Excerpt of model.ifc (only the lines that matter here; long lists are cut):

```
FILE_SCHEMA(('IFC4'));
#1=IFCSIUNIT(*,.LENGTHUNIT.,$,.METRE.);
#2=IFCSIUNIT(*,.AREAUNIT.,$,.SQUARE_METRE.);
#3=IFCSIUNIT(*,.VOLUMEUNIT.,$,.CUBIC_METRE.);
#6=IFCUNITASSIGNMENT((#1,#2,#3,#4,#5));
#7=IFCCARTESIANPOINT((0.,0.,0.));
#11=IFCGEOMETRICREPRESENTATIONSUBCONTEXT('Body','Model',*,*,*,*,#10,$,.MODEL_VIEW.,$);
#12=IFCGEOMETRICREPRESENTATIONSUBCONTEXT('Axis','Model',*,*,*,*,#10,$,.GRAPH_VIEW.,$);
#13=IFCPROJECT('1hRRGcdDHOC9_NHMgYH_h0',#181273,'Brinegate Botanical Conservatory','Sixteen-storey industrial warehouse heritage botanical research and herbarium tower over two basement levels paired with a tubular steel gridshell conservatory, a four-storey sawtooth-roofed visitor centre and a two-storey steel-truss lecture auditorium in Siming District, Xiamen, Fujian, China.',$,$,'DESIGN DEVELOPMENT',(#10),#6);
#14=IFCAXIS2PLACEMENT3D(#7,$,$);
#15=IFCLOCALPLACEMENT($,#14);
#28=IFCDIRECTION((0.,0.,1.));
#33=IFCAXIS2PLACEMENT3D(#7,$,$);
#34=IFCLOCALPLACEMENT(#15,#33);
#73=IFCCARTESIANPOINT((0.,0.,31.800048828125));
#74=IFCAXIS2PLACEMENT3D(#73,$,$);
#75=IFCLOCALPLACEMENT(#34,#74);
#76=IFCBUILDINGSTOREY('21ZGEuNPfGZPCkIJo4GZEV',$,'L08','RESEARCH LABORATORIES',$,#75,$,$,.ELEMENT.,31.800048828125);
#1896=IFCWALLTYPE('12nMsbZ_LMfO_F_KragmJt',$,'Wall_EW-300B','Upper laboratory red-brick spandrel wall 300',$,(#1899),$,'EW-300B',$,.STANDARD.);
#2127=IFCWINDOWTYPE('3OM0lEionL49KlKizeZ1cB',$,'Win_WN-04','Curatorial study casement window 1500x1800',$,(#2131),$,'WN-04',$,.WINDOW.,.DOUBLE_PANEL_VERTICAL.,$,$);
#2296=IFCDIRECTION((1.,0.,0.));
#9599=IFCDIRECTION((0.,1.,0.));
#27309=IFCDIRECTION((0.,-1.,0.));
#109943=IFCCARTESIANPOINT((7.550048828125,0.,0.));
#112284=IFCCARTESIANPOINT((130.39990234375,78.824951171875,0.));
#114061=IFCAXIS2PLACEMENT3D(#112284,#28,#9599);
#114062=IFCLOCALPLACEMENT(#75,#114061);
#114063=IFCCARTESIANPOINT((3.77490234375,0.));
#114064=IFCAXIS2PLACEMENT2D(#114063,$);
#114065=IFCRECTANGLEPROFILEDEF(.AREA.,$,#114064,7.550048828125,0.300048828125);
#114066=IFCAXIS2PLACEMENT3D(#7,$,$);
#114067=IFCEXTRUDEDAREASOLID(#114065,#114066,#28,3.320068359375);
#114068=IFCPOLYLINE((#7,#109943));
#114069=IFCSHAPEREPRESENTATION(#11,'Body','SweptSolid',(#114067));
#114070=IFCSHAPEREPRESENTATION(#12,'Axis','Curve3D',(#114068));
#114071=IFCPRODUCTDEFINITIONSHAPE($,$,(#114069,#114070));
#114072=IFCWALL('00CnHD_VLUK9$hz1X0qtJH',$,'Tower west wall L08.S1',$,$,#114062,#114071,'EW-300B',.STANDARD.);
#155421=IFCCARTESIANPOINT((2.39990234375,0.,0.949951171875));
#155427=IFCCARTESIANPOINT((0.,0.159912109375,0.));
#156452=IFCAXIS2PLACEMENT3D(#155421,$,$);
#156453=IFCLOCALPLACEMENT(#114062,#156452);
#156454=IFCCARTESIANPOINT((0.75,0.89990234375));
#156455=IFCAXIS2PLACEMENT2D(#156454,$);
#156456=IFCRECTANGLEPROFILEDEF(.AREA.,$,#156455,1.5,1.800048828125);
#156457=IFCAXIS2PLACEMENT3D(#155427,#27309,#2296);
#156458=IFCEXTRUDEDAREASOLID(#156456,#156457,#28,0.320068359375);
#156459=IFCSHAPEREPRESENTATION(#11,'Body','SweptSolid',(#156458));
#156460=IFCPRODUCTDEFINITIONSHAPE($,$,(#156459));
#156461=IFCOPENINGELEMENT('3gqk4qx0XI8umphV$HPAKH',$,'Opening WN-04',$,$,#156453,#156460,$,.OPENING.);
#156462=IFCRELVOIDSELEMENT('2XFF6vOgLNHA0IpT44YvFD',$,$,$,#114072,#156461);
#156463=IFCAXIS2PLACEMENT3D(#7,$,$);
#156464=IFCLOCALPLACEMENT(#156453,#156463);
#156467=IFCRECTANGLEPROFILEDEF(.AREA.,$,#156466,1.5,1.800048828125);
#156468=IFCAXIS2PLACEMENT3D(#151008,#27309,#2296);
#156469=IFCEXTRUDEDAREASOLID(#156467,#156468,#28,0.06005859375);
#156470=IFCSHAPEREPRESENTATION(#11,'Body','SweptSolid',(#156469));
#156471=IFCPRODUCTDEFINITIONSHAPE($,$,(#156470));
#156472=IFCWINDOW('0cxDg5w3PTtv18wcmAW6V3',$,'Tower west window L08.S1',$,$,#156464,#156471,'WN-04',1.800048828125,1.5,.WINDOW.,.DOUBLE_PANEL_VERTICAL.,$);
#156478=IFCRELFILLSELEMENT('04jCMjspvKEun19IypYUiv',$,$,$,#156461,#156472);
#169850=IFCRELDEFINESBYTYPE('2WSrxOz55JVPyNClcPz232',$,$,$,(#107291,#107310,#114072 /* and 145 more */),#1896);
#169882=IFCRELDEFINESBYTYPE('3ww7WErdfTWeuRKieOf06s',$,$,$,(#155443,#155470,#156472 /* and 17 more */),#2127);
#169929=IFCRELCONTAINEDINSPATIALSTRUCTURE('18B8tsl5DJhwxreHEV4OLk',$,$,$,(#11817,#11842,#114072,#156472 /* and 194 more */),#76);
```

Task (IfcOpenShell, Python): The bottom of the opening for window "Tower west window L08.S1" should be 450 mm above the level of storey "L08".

```python
import numpy as np
import ifcopenshell
import ifcopenshell.api.geometry
import ifcopenshell.geom
import ifcopenshell.util.element
import ifcopenshell.util.placement
import ifcopenshell.util.shape
import ifcopenshell.util.unit

model = ifcopenshell.open("model.ifc")
unit_scale = ifcopenshell.util.unit.calculate_unit_scale(model)

window = model.by_guid("0cxDg5w3PTtv18wcmAW6V3")
opening = window.FillsVoids[0].RelatingOpeningElement
storey = ifcopenshell.util.element.get_container(window, ifc_class="IfcBuildingStorey")
level = ifcopenshell.util.placement.get_local_placement(storey.ObjectPlacement)[2, 3]

# The opening's origin need not be at the sill, so measure its lowest point.
shape = ifcopenshell.geom.create_shape(ifcopenshell.geom.settings(), opening)
bottom = ifcopenshell.util.shape.get_shape_bottom_elevation(shape, shape.geometry) / unit_scale
dz = level + 0.45 - bottom

shift = np.array([0.0, 0.0, dz])
# The window is placed relative to its opening, so it follows when the opening moves.
matrix = ifcopenshell.util.placement.get_local_placement(opening.ObjectPlacement)
matrix[:3, 3] += shift
ifcopenshell.api.geometry.edit_object_placement(
    model, product=opening, matrix=matrix, is_si=False, should_transform_children=True
)

print(f"moved by {dz * unit_scale:+.3f} m")

model.write("model-out.ifc")
```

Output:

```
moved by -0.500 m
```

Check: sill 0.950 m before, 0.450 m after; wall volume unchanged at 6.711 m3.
